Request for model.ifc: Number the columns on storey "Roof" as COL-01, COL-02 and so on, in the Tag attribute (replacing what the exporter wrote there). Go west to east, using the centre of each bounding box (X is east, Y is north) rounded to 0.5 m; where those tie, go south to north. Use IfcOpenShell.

First a look at what the model holds.

```python
import ifcopenshell
import ifcopenshell.util.element
import ifcopenshell.util.placement

model = ifcopenshell.open("model.ifc")
print(model.schema)
storey = next(s for s in model.by_type("IfcBuildingStorey") if s.Name == "Roof")
columns = [e for e in ifcopenshell.util.element.get_decomposition(storey) if e.is_a("IfcColumn")]
for e in sorted(columns, key=lambda e: e.id()):
    origin = ifcopenshell.util.placement.get_local_placement(e.ObjectPlacement)[:3, 3]
    print(e.id(), e.Tag, e.Name, origin.round(2) + 0.0, sep=" | ")
```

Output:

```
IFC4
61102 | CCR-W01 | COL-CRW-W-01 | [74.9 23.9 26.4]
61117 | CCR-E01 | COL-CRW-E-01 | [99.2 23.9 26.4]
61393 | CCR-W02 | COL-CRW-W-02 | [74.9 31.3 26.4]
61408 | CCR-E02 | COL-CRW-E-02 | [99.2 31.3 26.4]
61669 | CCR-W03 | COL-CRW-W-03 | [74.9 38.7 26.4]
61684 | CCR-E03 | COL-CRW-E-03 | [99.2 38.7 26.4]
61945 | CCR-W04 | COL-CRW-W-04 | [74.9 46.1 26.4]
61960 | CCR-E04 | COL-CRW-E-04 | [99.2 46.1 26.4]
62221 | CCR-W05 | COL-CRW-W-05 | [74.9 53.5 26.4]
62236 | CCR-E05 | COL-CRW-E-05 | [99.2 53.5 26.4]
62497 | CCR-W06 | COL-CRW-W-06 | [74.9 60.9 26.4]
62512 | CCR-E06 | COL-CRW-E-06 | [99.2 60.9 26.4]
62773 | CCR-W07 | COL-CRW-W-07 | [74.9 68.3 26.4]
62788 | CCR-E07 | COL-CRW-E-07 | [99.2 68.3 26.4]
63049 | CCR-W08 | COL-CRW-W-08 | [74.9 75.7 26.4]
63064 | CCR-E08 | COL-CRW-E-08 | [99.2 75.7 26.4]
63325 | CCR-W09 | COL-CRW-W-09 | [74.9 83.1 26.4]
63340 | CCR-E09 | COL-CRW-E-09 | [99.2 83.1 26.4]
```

```python
import ifcopenshell
import ifcopenshell.geom
import ifcopenshell.util.element
import ifcopenshell.util.shape

model = ifcopenshell.open("model.ifc")
settings = ifcopenshell.geom.settings()
settings.set("use-world-coords", True)


def centre(element):
    shape = ifcopenshell.geom.create_shape(settings, element)
    return ifcopenshell.util.shape.get_bbox_centroid(shape.geometry)


storey = next(s for s in model.by_type("IfcBuildingStorey") if s.Name == "Roof")
columns = [e for e in ifcopenshell.util.element.get_decomposition(storey) if e.is_a("IfcColumn")]

# Insertion points can sit at a corner or the storey origin, so sort by the geometry (in metres).
centres = {e: centre(e) for e in columns}
columns.sort(key=lambda e: (round(centres[e][0] / 0.5), centres[e][1]))

for i, e in enumerate(columns, start=1):
    number = f"COL-{i:02d}"
    e.Tag = number
    print(e.id(), number)

model.write("model_v2.ifc")
```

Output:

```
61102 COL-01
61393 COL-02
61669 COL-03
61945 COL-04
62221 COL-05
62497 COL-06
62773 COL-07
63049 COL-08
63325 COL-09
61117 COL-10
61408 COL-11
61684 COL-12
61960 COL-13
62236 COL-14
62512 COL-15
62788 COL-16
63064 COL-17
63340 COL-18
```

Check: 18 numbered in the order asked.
